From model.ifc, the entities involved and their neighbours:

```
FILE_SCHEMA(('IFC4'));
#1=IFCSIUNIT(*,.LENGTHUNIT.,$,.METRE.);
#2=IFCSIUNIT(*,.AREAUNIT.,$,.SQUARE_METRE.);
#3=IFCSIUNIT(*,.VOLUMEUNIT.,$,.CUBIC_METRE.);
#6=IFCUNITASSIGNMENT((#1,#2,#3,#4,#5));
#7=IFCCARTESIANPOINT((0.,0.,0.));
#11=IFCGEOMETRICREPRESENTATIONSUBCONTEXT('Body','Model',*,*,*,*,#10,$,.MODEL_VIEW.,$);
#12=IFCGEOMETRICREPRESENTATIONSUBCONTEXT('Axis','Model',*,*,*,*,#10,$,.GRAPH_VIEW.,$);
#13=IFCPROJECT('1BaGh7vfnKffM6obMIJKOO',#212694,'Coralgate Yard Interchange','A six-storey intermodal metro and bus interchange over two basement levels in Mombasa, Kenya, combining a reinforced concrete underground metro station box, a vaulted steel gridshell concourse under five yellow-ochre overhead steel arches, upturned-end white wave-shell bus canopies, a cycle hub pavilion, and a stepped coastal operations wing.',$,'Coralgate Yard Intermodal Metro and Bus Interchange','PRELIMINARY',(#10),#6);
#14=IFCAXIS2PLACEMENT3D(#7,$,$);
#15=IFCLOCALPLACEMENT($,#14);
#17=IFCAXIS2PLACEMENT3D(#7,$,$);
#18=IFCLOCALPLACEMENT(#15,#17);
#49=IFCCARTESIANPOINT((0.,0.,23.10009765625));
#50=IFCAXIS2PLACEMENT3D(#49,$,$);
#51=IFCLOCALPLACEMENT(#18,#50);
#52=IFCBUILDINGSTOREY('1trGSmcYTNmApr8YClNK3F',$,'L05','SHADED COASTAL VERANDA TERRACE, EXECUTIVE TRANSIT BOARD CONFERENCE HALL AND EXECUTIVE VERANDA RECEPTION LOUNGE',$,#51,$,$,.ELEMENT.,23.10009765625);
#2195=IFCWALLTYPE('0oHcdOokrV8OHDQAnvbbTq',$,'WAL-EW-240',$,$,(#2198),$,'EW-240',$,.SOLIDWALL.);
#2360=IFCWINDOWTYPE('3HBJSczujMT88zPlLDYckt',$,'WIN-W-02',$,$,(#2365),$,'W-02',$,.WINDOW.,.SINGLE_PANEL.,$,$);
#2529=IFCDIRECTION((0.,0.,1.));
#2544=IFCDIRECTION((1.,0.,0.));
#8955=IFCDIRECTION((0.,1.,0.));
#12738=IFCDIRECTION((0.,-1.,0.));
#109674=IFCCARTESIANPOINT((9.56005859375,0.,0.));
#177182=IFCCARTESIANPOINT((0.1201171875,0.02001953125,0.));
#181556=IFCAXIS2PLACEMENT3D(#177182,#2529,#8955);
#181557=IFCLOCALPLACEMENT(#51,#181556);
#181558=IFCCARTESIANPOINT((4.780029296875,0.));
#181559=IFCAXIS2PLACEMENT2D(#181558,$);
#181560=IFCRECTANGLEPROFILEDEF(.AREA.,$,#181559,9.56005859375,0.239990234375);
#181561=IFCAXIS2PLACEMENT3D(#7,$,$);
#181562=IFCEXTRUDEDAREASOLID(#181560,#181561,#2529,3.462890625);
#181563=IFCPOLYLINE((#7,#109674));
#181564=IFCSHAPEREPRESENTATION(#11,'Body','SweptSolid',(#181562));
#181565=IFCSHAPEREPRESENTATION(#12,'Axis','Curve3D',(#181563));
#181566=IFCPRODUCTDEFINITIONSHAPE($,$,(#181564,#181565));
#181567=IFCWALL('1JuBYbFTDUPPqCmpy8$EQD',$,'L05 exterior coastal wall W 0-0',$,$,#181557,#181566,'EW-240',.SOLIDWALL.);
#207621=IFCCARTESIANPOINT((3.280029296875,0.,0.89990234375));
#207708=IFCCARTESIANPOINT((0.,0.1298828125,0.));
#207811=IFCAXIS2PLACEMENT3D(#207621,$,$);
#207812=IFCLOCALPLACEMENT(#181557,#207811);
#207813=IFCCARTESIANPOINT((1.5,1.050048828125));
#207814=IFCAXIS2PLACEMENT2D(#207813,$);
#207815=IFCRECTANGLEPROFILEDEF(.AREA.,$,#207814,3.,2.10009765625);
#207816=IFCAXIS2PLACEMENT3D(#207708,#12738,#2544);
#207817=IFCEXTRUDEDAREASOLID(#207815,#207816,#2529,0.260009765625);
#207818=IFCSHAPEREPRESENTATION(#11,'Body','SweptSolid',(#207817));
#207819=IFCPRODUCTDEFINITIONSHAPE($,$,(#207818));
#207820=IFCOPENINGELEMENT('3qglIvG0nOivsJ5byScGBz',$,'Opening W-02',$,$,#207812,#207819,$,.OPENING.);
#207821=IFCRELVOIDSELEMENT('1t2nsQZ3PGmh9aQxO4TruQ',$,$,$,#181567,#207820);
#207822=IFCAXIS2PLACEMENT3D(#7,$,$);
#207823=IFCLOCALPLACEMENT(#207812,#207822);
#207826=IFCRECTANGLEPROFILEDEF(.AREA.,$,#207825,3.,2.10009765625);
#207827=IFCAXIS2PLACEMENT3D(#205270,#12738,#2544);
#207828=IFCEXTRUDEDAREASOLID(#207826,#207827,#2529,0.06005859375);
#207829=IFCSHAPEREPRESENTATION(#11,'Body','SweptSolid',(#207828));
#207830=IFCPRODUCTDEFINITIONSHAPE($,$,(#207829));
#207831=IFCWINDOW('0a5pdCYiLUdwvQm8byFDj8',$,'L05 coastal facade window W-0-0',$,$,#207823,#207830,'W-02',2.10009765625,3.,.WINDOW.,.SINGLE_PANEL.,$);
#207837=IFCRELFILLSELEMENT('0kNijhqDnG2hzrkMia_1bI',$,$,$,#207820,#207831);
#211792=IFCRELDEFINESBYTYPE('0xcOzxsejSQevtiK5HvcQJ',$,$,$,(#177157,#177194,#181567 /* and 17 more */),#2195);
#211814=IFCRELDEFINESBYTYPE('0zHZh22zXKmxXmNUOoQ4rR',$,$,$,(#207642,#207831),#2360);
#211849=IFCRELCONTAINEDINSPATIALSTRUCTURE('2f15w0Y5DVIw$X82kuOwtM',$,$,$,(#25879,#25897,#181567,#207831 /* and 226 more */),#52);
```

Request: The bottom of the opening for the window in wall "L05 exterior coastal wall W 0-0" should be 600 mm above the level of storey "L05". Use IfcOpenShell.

```python
import numpy as np
import ifcopenshell
import ifcopenshell.api.geometry
import ifcopenshell.geom
import ifcopenshell.util.element
import ifcopenshell.util.placement
import ifcopenshell.util.shape
import ifcopenshell.util.unit

model = ifcopenshell.open("model.ifc")
unit_scale = ifcopenshell.util.unit.calculate_unit_scale(model)

window = model.by_guid("0a5pdCYiLUdwvQm8byFDj8")
opening = window.FillsVoids[0].RelatingOpeningElement
storey = ifcopenshell.util.element.get_container(window, ifc_class="IfcBuildingStorey")
level = ifcopenshell.util.placement.get_local_placement(storey.ObjectPlacement)[2, 3]

# The opening's origin need not be at the sill, so measure its lowest point.
shape = ifcopenshell.geom.create_shape(ifcopenshell.geom.settings(), opening)
bottom = ifcopenshell.util.shape.get_shape_bottom_elevation(shape, shape.geometry) / unit_scale
dz = level + 0.6 / unit_scale - bottom

shift = np.array([0.0, 0.0, dz])
# The window is placed relative to its opening, so it follows when the opening moves.
matrix = ifcopenshell.util.placement.get_local_placement(opening.ObjectPlacement)
matrix[:3, 3] += shift
ifcopenshell.api.geometry.edit_object_placement(
    model, product=opening, matrix=matrix, is_si=False, should_transform_children=True
)

print(f"moved by {dz * unit_scale:+.3f} m")

model.write("model_rev.ifc")
```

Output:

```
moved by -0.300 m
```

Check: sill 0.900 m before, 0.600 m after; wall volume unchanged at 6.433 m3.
